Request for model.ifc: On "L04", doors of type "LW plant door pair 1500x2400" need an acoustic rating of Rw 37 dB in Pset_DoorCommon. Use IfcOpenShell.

First a look at what the model holds.

```python
import ifcopenshell
import ifcopenshell.util.element

model = ifcopenshell.open("model.ifc")
print(model.schema)
storey = next(s for s in model.by_type("IfcBuildingStorey") if s.Name == "L04")
doors = [e for e in ifcopenshell.util.element.get_decomposition(storey) if e.is_a("IfcDoor")]
seen = {}
for e in doors:
    element_type = ifcopenshell.util.element.get_type(e)
    key = (element_type.Name if element_type != e and element_type else None, ifcopenshell.util.element.get_pset(e, "Pset_DoorCommon", "AcousticRating"))
    seen[key] = seen.get(key, 0) + 1
for (name, value), count in sorted(seen.items(), key=str):
    print(count, "x", name, "|", value)
```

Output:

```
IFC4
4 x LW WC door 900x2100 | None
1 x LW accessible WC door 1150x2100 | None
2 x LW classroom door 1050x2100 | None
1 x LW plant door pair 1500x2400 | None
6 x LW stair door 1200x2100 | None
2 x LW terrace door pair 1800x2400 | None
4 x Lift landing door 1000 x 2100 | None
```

```python
import ifcopenshell
import ifcopenshell.api.pset
import ifcopenshell.util.element

model = ifcopenshell.open("model.ifc")

storey = next(s for s in model.by_type("IfcBuildingStorey") if s.Name == "L04")
doors = [e for e in ifcopenshell.util.element.get_decomposition(storey) if e.is_a("IfcDoor")]

count = 0
for e in doors:
    element_type = ifcopenshell.util.element.get_type(e)
    if element_type in (None, e) or element_type.Name != "LW plant door pair 1500x2400":
        continue
    # add_pset returns the element's existing set when there is one.
    pset = ifcopenshell.api.pset.add_pset(model, product=e, name="Pset_DoorCommon")
    ifcopenshell.api.pset.edit_pset(model, pset=pset, properties={"AcousticRating": "Rw 37 dB"})
    count += 1

print(count, "doors updated")

model.write("model-out.ifc")
```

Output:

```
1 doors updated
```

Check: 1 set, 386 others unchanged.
